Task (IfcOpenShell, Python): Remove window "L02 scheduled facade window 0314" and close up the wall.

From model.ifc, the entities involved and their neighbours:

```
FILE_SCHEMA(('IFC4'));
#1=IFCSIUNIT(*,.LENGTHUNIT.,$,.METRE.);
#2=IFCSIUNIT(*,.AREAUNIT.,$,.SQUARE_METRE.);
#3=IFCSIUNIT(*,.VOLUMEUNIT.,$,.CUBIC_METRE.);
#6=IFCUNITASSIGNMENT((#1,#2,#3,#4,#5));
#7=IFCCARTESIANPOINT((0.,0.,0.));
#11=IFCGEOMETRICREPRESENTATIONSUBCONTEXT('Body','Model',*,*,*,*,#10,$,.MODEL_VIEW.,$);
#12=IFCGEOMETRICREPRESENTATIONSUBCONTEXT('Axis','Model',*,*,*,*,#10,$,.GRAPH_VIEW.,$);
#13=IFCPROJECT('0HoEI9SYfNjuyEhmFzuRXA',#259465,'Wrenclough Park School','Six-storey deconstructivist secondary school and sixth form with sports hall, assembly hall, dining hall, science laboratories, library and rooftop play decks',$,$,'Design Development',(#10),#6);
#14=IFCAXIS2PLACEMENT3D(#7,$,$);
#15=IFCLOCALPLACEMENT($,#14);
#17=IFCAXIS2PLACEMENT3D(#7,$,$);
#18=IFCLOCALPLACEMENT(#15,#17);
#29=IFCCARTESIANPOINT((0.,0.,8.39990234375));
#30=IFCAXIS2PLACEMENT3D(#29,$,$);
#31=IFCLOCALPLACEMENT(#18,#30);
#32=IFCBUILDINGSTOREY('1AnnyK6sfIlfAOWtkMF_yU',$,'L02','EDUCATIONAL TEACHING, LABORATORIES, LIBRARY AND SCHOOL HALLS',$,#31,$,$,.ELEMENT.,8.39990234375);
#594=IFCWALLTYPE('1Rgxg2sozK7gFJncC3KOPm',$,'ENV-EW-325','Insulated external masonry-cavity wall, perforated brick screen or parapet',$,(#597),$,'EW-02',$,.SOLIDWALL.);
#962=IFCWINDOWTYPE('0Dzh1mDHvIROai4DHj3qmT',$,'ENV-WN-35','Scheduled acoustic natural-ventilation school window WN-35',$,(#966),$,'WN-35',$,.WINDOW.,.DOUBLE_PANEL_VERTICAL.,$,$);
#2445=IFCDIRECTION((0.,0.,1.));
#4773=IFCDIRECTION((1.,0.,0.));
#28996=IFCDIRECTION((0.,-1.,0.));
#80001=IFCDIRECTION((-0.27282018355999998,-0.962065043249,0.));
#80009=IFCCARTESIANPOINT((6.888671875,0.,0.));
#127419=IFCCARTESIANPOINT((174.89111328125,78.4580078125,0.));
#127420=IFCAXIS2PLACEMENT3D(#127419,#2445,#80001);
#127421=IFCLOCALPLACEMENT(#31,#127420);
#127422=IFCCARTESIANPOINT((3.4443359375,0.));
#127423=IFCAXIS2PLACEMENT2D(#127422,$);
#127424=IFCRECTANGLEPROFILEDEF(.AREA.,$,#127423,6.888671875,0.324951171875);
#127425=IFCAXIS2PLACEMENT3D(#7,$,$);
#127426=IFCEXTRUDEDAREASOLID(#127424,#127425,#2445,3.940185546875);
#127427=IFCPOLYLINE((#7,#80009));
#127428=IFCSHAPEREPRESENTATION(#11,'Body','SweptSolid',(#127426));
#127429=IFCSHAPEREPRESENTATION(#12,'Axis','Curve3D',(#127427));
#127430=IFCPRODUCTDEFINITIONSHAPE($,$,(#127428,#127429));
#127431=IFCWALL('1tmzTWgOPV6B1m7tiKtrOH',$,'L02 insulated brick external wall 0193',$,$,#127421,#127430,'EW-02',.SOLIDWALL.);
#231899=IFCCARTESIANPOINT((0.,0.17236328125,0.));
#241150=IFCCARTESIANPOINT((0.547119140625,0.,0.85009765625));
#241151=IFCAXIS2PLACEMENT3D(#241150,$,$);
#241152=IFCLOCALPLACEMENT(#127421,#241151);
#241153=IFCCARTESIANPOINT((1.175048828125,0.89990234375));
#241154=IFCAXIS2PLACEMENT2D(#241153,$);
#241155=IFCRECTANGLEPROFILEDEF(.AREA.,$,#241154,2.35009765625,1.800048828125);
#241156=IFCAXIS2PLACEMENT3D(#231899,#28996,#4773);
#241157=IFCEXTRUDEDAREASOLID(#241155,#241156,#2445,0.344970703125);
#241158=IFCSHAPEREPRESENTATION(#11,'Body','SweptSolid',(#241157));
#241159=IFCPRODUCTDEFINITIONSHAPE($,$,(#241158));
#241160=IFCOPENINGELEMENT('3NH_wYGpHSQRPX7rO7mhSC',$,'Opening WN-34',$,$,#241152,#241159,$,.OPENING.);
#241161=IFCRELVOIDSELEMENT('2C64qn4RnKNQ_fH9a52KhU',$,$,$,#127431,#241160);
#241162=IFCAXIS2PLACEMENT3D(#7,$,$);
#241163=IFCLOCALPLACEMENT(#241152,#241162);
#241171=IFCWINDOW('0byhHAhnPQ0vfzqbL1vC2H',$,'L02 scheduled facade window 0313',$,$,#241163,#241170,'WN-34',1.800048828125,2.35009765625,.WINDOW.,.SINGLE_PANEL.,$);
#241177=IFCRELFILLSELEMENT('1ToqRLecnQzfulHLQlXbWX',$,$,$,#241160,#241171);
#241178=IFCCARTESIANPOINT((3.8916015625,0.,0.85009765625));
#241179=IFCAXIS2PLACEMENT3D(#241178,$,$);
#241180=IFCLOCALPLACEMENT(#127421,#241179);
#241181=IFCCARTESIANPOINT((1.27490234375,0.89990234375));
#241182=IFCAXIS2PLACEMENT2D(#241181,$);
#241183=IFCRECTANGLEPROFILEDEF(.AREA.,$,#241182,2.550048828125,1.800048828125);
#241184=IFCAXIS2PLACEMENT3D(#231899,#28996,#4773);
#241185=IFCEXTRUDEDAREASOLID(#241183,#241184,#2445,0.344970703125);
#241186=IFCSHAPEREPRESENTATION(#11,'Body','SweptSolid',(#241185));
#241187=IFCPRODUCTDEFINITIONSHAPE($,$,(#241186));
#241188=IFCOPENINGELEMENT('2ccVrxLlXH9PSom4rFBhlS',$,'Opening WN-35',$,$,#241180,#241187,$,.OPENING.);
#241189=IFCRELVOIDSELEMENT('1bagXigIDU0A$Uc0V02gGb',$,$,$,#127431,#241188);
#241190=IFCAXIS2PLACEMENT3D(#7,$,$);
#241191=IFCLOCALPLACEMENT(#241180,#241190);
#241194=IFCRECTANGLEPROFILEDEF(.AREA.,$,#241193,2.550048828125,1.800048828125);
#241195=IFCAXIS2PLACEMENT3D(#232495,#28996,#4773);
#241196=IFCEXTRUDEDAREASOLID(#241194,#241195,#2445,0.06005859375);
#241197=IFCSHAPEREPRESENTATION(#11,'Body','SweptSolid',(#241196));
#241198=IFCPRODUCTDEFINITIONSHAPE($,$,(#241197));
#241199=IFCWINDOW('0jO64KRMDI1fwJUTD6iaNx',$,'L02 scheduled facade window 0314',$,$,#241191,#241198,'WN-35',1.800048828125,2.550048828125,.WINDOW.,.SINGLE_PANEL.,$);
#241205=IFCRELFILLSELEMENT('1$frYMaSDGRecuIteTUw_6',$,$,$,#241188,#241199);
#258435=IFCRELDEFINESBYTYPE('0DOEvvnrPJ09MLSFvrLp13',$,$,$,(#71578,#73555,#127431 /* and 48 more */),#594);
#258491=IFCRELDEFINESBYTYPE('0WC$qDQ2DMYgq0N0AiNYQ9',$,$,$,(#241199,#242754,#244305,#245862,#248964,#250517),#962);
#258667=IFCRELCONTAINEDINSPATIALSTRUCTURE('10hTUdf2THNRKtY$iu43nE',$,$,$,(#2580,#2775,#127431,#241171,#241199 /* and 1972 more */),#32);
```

```python
import ifcopenshell
import ifcopenshell.api.feature
import ifcopenshell.api.root
import ifcopenshell.geom
import ifcopenshell.util.shape

model = ifcopenshell.open("model.ifc")
settings = ifcopenshell.geom.settings()


def volume(element):
    """Net volume in cubic metres, openings subtracted."""
    shape = ifcopenshell.geom.create_shape(settings, element)
    return ifcopenshell.util.shape.get_volume(shape.geometry)


window = model.by_guid("0jO64KRMDI1fwJUTD6iaNx")
opening = window.FillsVoids[0].RelatingOpeningElement
wall = opening.VoidsElements[0].RelatingBuildingElement
before = volume(wall)

ifcopenshell.api.root.remove_product(model, product=window)
ifcopenshell.api.feature.remove_feature(model, feature=opening)

after = volume(wall)

print(f"wall volume {before:.3f} -> {after:.3f} m3")

model.write("model_updated.ifc")
```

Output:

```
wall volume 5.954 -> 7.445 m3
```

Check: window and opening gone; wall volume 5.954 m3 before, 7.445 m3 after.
